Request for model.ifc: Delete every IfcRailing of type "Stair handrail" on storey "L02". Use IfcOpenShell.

First a look at what the model holds.

```python
import ifcopenshell
import ifcopenshell.util.element

model = ifcopenshell.open("model.ifc")
print(model.schema)
storey = next(s for s in model.by_type("IfcBuildingStorey") if s.Name == "L02")
railings = [e for e in ifcopenshell.util.element.get_decomposition(storey) if e.is_a("IfcRailing")]
seen = {}
for e in railings:
    element_type = ifcopenshell.util.element.get_type(e)
    name = element_type.Name if element_type not in (None, e) else None
    seen[name] = seen.get(name, 0) + 1
for name, count in sorted(seen.items(), key=str):
    print(count, "x", name)
```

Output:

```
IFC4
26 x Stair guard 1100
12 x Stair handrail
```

```python
import ifcopenshell
import ifcopenshell.api.root
import ifcopenshell.util.element

model = ifcopenshell.open("model.ifc")

storey = next(s for s in model.by_type("IfcBuildingStorey") if s.Name == "L02")
railings = [e for e in ifcopenshell.util.element.get_decomposition(storey) if e.is_a("IfcRailing")]
targets = [e for e in railings if (t := ifcopenshell.util.element.get_type(e)) not in (None, e) and t.Name == "Stair handrail"]

for e in targets:
    ifcopenshell.api.root.remove_product(model, product=e)
print(len(targets), "removed")

model.write("model_v2.ifc")
```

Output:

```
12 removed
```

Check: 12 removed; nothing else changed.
